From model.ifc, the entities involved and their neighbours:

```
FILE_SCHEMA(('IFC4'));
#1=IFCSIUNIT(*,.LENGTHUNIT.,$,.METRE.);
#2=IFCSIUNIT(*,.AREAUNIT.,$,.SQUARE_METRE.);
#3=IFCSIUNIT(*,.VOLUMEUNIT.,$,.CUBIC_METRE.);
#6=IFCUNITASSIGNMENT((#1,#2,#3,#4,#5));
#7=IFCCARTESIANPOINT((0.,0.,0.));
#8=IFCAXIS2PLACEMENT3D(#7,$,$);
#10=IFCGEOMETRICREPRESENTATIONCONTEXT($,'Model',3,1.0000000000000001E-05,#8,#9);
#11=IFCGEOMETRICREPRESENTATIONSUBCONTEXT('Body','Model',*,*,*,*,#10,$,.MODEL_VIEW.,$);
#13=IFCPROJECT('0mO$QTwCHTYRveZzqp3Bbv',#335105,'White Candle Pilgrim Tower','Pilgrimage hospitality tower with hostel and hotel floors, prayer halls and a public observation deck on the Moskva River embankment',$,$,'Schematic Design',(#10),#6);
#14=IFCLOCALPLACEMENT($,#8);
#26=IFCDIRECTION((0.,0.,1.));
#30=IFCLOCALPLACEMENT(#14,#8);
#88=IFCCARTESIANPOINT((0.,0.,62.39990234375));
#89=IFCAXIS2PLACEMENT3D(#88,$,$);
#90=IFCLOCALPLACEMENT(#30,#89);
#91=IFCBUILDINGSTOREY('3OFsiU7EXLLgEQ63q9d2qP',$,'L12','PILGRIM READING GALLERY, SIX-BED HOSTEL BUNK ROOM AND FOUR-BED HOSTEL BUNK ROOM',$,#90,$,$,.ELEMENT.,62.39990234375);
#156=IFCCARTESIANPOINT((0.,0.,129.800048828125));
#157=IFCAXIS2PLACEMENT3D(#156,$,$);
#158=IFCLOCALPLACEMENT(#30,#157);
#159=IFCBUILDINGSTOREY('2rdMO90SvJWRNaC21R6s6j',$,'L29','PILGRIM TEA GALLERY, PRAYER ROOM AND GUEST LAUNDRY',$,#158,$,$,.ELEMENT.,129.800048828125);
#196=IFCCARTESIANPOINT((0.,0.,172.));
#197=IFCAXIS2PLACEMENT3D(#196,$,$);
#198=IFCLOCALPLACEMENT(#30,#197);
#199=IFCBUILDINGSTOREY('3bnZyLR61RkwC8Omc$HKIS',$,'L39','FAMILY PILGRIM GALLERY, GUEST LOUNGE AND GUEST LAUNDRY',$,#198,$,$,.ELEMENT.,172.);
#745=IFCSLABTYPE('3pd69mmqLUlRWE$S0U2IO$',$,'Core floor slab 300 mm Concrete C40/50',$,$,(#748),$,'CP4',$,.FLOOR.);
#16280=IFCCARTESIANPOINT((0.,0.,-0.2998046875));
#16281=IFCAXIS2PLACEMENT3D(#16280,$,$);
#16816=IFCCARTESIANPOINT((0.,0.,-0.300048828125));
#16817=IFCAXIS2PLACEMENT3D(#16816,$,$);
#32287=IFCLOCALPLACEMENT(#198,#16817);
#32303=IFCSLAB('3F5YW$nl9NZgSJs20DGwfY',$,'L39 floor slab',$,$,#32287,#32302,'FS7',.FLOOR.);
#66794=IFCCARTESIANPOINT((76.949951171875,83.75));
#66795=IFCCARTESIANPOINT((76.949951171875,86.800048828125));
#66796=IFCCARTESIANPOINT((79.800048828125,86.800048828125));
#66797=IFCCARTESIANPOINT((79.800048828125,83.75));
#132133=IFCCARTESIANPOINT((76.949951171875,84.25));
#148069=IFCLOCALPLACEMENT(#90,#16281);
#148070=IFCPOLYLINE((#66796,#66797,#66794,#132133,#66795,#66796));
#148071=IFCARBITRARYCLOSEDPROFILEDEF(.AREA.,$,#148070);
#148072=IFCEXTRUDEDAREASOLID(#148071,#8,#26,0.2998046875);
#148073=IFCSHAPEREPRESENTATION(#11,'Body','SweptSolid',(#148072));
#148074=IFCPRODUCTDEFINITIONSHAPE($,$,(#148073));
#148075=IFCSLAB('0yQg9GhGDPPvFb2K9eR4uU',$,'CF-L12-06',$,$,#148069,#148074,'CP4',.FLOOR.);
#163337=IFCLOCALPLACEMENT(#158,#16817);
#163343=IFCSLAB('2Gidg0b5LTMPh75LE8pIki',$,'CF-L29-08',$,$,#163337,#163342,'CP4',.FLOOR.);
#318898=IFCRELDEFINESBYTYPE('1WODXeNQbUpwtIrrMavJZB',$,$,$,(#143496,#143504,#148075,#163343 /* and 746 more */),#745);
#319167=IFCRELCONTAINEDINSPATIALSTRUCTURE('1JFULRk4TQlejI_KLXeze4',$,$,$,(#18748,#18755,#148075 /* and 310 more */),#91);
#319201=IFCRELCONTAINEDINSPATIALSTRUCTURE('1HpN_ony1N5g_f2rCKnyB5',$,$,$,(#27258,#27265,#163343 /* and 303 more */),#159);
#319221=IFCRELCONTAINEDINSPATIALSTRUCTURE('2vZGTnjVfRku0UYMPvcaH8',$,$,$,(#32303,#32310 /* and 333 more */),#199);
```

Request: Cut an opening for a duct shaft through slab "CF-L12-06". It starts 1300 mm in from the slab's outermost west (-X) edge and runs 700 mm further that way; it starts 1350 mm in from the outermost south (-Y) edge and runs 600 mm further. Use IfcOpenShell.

```python
import numpy as np
import ifcopenshell
import ifcopenshell.api.feature
import ifcopenshell.api.geometry
import ifcopenshell.api.root
import ifcopenshell.geom
import ifcopenshell.util.placement
import ifcopenshell.util.representation
import ifcopenshell.util.shape
import ifcopenshell.util.unit

model = ifcopenshell.open("model.ifc")
unit_scale = ifcopenshell.util.unit.calculate_unit_scale(model)
settings = ifcopenshell.geom.settings()


def volume(element):
    """Net volume in cubic metres, openings subtracted."""
    shape = ifcopenshell.geom.create_shape(settings, element)
    return ifcopenshell.util.shape.get_volume(shape.geometry)


slab = model.by_guid("0yQg9GhGDPPvFb2K9eR4uU")
before = volume(slab)

# Extent in the slab's own axes, in metres. The edges named are its -X and -Y sides.
slab_shape = ifcopenshell.geom.create_shape(settings, slab)
vertices = ifcopenshell.util.shape.get_vertices(slab_shape.geometry)
x_min, y_min, bottom = vertices.min(axis=0)
top = vertices[:, 2].max()

opening = ifcopenshell.api.root.create_entity(model, ifc_class="IfcOpeningElement", name="Duct shaft opening", predefined_type="OPENING")
context = ifcopenshell.util.representation.get_context(model, "Model", "Body", "MODEL_VIEW")
width, depth = 0.7, 0.6
outline = [(0.0, 0.0), (width, 0.0), (width, depth), (0.0, depth), (0.0, 0.0)]
# Overshoot both faces by 50 mm so the cut is clean.
shape = ifcopenshell.api.geometry.add_slab_representation(
    model, context=context, depth=top - bottom + 0.1, polyline=outline
)
ifcopenshell.api.geometry.assign_representation(model, product=opening, representation=shape)

matrix = ifcopenshell.util.placement.get_local_placement(slab.ObjectPlacement)
matrix[:, 3] = matrix @ np.append(np.array([x_min + 1.3, y_min + 1.35, bottom - 0.05]) / unit_scale, 1.0)
ifcopenshell.api.geometry.edit_object_placement(model, product=opening, matrix=matrix, is_si=False)
ifcopenshell.api.feature.add_feature(model, feature=opening, element=slab)

after = volume(slab)

print(f"slab volume {before:.3f} -> {after:.3f} m3")

model.write("model_v2.ifc")
```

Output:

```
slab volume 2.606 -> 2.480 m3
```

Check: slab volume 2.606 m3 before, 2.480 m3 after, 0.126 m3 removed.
